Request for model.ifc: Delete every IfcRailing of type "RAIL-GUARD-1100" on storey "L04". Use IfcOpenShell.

First a look at what the model holds.

```python
import ifcopenshell
import ifcopenshell.util.element

model = ifcopenshell.open("model.ifc")
print(model.schema)
storey = next(s for s in model.by_type("IfcBuildingStorey") if s.Name == "L04")
railings = [e for e in ifcopenshell.util.element.get_decomposition(storey) if e.is_a("IfcRailing")]
seen = {}
for e in railings:
    element_type = ifcopenshell.util.element.get_type(e)
    name = element_type.Name if element_type not in (None, e) else None
    seen[name] = seen.get(name, 0) + 1
for name, count in sorted(seen.items(), key=str):
    print(count, "x", name)
```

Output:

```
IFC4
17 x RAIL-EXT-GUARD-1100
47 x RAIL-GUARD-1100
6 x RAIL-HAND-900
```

```python
import ifcopenshell
import ifcopenshell.api.root
import ifcopenshell.util.element

model = ifcopenshell.open("model.ifc")

storey = next(s for s in model.by_type("IfcBuildingStorey") if s.Name == "L04")
railings = [e for e in ifcopenshell.util.element.get_decomposition(storey) if e.is_a("IfcRailing")]
targets = [e for e in railings if (t := ifcopenshell.util.element.get_type(e)) not in (None, e) and t.Name == "RAIL-GUARD-1100"]

for e in targets:
    ifcopenshell.api.root.remove_product(model, product=e)
print(len(targets), "removed")

model.write("model_v2.ifc")
```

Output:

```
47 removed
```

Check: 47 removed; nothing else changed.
